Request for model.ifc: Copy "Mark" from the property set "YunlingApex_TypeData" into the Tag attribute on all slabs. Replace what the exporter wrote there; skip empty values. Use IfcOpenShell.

First a look at what the model holds.

```python
import ifcopenshell
import ifcopenshell.util.element

model = ifcopenshell.open("model.ifc")
print(model.schema)
slabs = model.by_type("IfcSlab")
print(len(slabs), "slabs")
for e in slabs[:8]:
    source = ifcopenshell.util.element.get_pset(e, "YunlingApex_TypeData", "Mark")
    target = e.Tag
    print(e.id(), repr(source), repr(target), sep=" | ")
```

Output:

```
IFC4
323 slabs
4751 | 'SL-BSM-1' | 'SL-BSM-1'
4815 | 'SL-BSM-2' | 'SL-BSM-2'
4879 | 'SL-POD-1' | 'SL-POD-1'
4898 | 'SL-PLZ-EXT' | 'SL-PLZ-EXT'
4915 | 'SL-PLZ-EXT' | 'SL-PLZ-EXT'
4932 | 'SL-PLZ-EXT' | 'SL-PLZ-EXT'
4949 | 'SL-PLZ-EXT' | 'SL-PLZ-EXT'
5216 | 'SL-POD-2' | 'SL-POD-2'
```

```python
import ifcopenshell
import ifcopenshell.util.element

model = ifcopenshell.open("model.ifc")

count = 0
for e in model.by_type("IfcSlab"):
    value = ifcopenshell.util.element.get_pset(e, "YunlingApex_TypeData", "Mark")
    current = e.Tag
    if not value or not value.strip() or current == value:
        continue
    e.Tag = value
    count += 1

print(count, "slabs updated")

model.write("model_updated.ifc")
```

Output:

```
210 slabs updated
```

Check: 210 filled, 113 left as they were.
